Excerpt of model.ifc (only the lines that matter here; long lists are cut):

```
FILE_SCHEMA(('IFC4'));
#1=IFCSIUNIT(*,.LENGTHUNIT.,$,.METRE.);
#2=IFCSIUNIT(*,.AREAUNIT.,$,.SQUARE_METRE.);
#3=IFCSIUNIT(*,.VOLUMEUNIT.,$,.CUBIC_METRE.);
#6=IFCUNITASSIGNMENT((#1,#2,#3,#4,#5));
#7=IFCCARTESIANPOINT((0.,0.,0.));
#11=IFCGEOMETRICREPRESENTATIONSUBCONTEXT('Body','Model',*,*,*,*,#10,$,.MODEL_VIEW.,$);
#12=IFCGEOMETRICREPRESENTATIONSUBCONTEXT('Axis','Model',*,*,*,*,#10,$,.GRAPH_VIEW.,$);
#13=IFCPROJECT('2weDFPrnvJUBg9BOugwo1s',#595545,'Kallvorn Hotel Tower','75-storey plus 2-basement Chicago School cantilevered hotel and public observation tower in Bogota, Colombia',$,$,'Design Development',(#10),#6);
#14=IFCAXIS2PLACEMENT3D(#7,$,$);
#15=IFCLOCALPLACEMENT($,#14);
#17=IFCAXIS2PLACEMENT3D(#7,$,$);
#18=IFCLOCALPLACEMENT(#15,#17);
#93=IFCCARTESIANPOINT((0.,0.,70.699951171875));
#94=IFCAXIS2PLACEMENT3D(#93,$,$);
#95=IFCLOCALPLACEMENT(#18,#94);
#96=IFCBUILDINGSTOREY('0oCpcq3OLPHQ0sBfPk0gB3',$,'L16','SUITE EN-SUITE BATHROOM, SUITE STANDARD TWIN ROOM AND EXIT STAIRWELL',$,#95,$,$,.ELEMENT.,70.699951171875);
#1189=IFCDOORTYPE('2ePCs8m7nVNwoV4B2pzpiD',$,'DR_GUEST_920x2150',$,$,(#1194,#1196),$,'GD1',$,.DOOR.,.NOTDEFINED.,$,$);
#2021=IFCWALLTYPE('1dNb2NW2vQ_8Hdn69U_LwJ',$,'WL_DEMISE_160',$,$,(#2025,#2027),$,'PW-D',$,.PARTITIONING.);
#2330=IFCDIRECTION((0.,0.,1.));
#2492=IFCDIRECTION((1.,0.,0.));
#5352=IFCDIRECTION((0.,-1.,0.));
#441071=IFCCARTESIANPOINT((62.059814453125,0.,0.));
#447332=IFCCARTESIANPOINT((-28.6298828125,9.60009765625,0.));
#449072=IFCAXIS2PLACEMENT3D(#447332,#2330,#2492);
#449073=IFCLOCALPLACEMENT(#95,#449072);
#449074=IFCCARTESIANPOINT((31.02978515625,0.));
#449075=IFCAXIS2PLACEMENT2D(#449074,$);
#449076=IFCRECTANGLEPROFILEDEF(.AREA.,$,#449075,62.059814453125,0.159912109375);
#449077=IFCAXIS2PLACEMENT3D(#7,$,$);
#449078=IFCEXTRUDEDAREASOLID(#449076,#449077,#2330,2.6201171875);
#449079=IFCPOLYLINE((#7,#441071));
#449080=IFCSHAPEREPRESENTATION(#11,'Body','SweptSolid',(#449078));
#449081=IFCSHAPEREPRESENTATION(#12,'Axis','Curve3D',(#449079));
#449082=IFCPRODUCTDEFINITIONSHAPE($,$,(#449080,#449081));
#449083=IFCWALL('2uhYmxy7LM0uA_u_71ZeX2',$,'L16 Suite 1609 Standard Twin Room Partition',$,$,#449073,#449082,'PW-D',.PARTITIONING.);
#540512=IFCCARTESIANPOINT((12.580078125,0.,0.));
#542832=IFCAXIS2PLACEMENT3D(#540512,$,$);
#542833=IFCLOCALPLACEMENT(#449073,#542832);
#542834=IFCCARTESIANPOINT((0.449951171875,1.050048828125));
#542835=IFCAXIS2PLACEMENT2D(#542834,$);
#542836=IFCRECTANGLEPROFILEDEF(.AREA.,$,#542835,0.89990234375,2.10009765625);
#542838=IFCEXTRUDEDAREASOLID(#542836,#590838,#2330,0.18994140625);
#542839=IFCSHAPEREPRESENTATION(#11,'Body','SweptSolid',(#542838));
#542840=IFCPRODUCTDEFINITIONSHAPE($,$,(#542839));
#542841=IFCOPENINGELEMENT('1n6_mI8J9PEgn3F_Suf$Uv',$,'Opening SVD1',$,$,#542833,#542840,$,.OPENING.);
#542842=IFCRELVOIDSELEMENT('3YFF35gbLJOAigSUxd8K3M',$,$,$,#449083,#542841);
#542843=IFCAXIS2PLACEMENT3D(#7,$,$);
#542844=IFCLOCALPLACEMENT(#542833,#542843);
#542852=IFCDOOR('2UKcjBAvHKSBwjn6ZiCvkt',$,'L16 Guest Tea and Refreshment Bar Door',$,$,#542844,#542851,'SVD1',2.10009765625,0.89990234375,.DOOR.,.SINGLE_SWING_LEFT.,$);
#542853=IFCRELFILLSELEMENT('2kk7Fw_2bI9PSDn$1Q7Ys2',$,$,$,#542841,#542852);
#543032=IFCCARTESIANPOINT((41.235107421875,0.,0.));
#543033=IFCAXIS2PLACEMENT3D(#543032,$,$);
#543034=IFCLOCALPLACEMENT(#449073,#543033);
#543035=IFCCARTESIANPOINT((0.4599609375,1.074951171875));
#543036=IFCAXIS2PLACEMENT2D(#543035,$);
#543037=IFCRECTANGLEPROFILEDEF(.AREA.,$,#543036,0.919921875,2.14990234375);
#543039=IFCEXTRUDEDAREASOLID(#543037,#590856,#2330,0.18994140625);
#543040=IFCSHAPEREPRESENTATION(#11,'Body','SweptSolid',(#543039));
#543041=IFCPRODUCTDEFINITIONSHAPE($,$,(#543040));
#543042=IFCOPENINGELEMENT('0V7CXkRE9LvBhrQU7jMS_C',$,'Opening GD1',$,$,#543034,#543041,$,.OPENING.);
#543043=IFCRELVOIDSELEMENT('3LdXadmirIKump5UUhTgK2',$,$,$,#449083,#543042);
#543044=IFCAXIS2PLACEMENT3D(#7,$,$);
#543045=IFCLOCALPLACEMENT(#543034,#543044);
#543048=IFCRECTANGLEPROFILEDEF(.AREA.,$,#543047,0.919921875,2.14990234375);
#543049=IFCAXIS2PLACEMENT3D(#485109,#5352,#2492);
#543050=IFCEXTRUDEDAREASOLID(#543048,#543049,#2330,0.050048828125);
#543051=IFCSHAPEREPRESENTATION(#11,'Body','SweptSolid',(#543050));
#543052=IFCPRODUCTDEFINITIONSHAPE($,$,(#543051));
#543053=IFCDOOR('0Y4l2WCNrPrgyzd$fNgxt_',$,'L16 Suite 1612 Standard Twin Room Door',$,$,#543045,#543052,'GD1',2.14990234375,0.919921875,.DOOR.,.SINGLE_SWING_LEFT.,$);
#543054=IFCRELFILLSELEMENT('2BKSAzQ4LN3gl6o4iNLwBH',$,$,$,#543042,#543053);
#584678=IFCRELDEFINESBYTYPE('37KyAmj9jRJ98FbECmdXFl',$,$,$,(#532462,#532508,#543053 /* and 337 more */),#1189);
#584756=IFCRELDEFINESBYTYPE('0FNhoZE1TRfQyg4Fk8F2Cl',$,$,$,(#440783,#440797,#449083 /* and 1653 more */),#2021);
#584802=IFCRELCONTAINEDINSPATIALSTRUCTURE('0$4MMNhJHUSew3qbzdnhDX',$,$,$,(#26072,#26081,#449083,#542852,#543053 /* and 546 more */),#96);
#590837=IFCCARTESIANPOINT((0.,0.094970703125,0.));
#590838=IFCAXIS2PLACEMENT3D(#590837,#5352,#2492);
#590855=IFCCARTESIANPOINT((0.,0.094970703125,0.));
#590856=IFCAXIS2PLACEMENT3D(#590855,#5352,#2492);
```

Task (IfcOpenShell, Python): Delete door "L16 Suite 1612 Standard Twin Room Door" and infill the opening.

```python
import ifcopenshell
import ifcopenshell.api.feature
import ifcopenshell.api.root
import ifcopenshell.geom
import ifcopenshell.util.shape

model = ifcopenshell.open("model.ifc")
settings = ifcopenshell.geom.settings()


def volume(element):
    """Net volume in cubic metres, openings subtracted."""
    shape = ifcopenshell.geom.create_shape(settings, element)
    return ifcopenshell.util.shape.get_volume(shape.geometry)


door = model.by_id(543053)
opening = door.FillsVoids[0].RelatingOpeningElement
wall = opening.VoidsElements[0].RelatingBuildingElement
before = volume(wall)

ifcopenshell.api.root.remove_product(model, product=door)
ifcopenshell.api.feature.remove_feature(model, feature=opening)

after = volume(wall)

print(f"wall volume {before:.3f} -> {after:.3f} m3")

model.write("model-out.ifc")
```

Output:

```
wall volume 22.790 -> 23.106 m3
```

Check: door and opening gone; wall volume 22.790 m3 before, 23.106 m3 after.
